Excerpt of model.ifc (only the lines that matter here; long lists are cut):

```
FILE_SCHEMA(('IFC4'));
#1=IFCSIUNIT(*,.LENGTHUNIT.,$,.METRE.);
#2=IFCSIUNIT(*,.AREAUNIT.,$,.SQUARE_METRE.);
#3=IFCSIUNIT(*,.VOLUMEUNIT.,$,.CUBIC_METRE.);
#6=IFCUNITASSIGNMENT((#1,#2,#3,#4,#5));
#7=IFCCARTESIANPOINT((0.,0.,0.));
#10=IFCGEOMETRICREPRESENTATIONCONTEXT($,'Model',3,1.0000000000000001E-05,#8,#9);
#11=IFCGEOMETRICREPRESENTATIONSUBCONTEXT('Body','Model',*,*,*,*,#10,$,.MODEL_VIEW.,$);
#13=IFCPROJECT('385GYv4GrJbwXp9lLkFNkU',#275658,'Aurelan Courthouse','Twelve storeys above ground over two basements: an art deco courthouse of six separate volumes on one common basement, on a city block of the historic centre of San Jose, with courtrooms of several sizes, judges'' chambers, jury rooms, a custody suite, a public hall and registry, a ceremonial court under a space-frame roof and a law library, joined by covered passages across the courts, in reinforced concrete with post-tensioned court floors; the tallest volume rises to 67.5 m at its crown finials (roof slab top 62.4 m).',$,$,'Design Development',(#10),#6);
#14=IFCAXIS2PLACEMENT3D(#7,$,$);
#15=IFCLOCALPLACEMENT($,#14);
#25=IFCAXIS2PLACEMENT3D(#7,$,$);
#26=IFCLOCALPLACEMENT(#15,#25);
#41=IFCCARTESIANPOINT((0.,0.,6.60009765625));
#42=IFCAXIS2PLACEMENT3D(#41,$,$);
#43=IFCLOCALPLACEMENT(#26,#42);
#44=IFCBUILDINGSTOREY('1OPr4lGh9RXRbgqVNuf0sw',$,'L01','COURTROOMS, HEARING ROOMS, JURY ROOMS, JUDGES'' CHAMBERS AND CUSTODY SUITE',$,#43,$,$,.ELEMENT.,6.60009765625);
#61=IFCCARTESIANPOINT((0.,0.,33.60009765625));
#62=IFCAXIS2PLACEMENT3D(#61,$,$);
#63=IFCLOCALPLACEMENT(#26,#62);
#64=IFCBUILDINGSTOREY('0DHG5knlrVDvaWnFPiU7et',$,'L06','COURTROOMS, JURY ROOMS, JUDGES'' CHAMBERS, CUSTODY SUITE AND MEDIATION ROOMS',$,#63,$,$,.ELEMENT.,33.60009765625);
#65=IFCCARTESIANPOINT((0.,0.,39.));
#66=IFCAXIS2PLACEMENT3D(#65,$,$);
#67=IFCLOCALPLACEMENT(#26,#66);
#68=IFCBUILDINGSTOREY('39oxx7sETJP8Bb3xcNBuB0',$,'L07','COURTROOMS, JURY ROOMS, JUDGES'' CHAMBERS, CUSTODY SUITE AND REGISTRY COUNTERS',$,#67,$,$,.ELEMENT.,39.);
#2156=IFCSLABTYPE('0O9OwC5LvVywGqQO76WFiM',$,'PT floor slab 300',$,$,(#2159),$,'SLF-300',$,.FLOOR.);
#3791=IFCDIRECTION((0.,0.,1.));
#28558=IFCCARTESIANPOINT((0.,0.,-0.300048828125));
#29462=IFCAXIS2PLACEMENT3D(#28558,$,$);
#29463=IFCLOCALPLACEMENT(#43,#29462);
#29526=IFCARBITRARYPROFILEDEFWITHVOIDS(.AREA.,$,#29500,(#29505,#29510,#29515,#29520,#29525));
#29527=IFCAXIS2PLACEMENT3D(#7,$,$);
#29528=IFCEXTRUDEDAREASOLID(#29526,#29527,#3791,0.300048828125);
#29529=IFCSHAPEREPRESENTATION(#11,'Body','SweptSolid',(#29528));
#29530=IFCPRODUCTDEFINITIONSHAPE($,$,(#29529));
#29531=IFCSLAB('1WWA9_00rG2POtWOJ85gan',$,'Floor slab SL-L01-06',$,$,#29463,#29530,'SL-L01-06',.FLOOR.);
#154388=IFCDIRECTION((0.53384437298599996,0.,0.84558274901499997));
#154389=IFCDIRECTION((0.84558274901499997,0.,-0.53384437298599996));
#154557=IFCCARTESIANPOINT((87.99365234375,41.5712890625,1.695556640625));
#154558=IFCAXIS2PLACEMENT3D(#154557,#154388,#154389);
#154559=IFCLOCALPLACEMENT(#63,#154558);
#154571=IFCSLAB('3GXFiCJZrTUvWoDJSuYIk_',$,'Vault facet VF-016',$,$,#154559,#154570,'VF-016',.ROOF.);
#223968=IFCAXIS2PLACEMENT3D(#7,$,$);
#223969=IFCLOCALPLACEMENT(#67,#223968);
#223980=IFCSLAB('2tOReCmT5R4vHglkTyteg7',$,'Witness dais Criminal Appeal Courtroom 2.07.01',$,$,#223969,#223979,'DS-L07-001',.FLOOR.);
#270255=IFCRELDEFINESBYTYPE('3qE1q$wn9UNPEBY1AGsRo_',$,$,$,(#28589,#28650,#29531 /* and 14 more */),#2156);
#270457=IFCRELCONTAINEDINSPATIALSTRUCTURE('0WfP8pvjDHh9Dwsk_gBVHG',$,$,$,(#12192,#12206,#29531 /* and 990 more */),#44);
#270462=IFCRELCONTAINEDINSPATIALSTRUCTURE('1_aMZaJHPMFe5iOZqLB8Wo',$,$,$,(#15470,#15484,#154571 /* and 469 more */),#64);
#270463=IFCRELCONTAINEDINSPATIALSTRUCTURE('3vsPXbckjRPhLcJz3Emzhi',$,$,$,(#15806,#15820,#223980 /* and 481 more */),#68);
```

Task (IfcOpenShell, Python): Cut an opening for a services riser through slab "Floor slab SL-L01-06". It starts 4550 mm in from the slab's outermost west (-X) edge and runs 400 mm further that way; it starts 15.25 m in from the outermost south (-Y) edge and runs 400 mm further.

```python
import numpy as np
import ifcopenshell
import ifcopenshell.api.feature
import ifcopenshell.api.geometry
import ifcopenshell.api.root
import ifcopenshell.geom
import ifcopenshell.util.placement
import ifcopenshell.util.representation
import ifcopenshell.util.shape
import ifcopenshell.util.unit

model = ifcopenshell.open("model.ifc")
unit_scale = ifcopenshell.util.unit.calculate_unit_scale(model)
settings = ifcopenshell.geom.settings()


def volume(element):
    """Net volume in cubic metres, openings subtracted."""
    shape = ifcopenshell.geom.create_shape(settings, element)
    return ifcopenshell.util.shape.get_volume(shape.geometry)


slab = model.by_id(29531)
before = volume(slab)

# Extent in the slab's own axes, in metres. The edges named are its -X and -Y sides.
slab_shape = ifcopenshell.geom.create_shape(settings, slab)
vertices = ifcopenshell.util.shape.get_vertices(slab_shape.geometry)
x_min, y_min, bottom = vertices.min(axis=0)
top = vertices[:, 2].max()

opening = ifcopenshell.api.root.create_entity(model, ifc_class="IfcOpeningElement", name="Services riser opening", predefined_type="OPENING")
context = ifcopenshell.util.representation.get_context(model, "Model", "Body", "MODEL_VIEW")
width, depth = 0.4, 0.4
outline = [(0.0, 0.0), (width, 0.0), (width, depth), (0.0, depth), (0.0, 0.0)]
# Overshoot both faces by 50 mm so the cut is clean.
shape = ifcopenshell.api.geometry.add_slab_representation(
    model, context=context, depth=top - bottom + 0.1, polyline=outline
)
ifcopenshell.api.geometry.assign_representation(model, product=opening, representation=shape)

matrix = ifcopenshell.util.placement.get_local_placement(slab.ObjectPlacement)
matrix[:, 3] = matrix @ np.append(np.array([x_min + 4.55, y_min + 15.25, bottom - 0.05]) / unit_scale, 1.0)
ifcopenshell.api.geometry.edit_object_placement(model, product=opening, matrix=matrix, is_si=False)
ifcopenshell.api.feature.add_feature(model, feature=opening, element=slab)

after = volume(slab)

print(f"slab volume {before:.3f} -> {after:.3f} m3")

model.write("model_v2.ifc")
```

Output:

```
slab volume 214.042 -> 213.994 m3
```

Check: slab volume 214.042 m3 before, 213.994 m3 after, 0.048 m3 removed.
